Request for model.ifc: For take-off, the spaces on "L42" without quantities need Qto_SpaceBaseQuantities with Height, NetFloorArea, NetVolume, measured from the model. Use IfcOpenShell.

First a look at what the model holds.

```python
import ifcopenshell
import ifcopenshell.util.element
import ifcopenshell.util.unit

model = ifcopenshell.open("model.ifc")
print(model.schema)
for unit_type in ("LENGTHUNIT", "AREAUNIT", "VOLUMEUNIT"):
    print(unit_type, ifcopenshell.util.unit.calculate_unit_scale(model, unit_type))
storey = next(s for s in model.by_type("IfcBuildingStorey") if s.Name == "L42")
spaces = [e for e in ifcopenshell.util.element.get_decomposition(storey) if e.is_a("IfcSpace")]
for e in sorted(spaces, key=lambda e: e.id()):
    print(e.id(), e.is_a(), e.Name, list(ifcopenshell.util.element.get_psets(e, qtos_only=True)), sep=" | ")
```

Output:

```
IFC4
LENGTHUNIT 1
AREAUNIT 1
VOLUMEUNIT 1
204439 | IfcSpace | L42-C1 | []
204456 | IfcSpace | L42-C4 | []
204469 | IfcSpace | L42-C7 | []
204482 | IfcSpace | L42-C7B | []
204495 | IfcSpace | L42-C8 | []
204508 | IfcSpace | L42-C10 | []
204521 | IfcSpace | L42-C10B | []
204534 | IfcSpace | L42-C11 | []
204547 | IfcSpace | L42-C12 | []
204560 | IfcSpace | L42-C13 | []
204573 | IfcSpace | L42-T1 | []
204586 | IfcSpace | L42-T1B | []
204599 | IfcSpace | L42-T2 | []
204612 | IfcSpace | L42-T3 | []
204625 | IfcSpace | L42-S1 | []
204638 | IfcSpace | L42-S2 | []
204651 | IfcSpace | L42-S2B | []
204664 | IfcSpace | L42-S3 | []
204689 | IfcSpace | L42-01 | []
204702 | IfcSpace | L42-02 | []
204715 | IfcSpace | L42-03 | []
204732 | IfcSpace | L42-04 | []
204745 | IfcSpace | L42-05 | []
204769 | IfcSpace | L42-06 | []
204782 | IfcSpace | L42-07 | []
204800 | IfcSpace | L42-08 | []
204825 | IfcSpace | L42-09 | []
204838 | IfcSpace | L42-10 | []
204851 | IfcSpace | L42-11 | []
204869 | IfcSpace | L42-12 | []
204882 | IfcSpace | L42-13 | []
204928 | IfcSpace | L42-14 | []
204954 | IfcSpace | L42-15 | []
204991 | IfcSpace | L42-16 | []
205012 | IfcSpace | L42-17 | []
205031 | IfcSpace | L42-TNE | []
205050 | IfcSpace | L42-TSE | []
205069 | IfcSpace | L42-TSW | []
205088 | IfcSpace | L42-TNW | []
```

```python
import ifcopenshell
import ifcopenshell.api.pset
import ifcopenshell.geom
import ifcopenshell.util.element
import ifcopenshell.util.shape
import ifcopenshell.util.unit

model = ifcopenshell.open("model.ifc")
unit_scale = ifcopenshell.util.unit.calculate_unit_scale(model)
area_scale = ifcopenshell.util.unit.calculate_unit_scale(model, "AREAUNIT")
volume_scale = ifcopenshell.util.unit.calculate_unit_scale(model, "VOLUMEUNIT")
settings = ifcopenshell.geom.settings()

storey = next(s for s in model.by_type("IfcBuildingStorey") if s.Name == "L42")
spaces = [e for e in ifcopenshell.util.element.get_decomposition(storey) if e.is_a("IfcSpace")]

for e in sorted(spaces, key=lambda e: e.id()):
    if ifcopenshell.util.element.get_psets(e, qtos_only=True, should_inherit=False):
        continue
    # Geometry comes back in metres, in the element's own axes.
    shape = ifcopenshell.geom.create_shape(settings, e)
    values = {
        "Height": ifcopenshell.util.shape.get_z(shape.geometry) / unit_scale,
        "NetFloorArea": ifcopenshell.util.shape.get_footprint_area(shape.geometry) / area_scale,
        "NetVolume": ifcopenshell.util.shape.get_volume(shape.geometry) / volume_scale,
    }
    qto = ifcopenshell.api.pset.add_qto(model, product=e, name="Qto_SpaceBaseQuantities")
    ifcopenshell.api.pset.edit_qto(model, qto=qto, properties=values)
    print(e.id(), {k: round(v, 3) for k, v in values.items()})

model.write("model_edited.ifc")
```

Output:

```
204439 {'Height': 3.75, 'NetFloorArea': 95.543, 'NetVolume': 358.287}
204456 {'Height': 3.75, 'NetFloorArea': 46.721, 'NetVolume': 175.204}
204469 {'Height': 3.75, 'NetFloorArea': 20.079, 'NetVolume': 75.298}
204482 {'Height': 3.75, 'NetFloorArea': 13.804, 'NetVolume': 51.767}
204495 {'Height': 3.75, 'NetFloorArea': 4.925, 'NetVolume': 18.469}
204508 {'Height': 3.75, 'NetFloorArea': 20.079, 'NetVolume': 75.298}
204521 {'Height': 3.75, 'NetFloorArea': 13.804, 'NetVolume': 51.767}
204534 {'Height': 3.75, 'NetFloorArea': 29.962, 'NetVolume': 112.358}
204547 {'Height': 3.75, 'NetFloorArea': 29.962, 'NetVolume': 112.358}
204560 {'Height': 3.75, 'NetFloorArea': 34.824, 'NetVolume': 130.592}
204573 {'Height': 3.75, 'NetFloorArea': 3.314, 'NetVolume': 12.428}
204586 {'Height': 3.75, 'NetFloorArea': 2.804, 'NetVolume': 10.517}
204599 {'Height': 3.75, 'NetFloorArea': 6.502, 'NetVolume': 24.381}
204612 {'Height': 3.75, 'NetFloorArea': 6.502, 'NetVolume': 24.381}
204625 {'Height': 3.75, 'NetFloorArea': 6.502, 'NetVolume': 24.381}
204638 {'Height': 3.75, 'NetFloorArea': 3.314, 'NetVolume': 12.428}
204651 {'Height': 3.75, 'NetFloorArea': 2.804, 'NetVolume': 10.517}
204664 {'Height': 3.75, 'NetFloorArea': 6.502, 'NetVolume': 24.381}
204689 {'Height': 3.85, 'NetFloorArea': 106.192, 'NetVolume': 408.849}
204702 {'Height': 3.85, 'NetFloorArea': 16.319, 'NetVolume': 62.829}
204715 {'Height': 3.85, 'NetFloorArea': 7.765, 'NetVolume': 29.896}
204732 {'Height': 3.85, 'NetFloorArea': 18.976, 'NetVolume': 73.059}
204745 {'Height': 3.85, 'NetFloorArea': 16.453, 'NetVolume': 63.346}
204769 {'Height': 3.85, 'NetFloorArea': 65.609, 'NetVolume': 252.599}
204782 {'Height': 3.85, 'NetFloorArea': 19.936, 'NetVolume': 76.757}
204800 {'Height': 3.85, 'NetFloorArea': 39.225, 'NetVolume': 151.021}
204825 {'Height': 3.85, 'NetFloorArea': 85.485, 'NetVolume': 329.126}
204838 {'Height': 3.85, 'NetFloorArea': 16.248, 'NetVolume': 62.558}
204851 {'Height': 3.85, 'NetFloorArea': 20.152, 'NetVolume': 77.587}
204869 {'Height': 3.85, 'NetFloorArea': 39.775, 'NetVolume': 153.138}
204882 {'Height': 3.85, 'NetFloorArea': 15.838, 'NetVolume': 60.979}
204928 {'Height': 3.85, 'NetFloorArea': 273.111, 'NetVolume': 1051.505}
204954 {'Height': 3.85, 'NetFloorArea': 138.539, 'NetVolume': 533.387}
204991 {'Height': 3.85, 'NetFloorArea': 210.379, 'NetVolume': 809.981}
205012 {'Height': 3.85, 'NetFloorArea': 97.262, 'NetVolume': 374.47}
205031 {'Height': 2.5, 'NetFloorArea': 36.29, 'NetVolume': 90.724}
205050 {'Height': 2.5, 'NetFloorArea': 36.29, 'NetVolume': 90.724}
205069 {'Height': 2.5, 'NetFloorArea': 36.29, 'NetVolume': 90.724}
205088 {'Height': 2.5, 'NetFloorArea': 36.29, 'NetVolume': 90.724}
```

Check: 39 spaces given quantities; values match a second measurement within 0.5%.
